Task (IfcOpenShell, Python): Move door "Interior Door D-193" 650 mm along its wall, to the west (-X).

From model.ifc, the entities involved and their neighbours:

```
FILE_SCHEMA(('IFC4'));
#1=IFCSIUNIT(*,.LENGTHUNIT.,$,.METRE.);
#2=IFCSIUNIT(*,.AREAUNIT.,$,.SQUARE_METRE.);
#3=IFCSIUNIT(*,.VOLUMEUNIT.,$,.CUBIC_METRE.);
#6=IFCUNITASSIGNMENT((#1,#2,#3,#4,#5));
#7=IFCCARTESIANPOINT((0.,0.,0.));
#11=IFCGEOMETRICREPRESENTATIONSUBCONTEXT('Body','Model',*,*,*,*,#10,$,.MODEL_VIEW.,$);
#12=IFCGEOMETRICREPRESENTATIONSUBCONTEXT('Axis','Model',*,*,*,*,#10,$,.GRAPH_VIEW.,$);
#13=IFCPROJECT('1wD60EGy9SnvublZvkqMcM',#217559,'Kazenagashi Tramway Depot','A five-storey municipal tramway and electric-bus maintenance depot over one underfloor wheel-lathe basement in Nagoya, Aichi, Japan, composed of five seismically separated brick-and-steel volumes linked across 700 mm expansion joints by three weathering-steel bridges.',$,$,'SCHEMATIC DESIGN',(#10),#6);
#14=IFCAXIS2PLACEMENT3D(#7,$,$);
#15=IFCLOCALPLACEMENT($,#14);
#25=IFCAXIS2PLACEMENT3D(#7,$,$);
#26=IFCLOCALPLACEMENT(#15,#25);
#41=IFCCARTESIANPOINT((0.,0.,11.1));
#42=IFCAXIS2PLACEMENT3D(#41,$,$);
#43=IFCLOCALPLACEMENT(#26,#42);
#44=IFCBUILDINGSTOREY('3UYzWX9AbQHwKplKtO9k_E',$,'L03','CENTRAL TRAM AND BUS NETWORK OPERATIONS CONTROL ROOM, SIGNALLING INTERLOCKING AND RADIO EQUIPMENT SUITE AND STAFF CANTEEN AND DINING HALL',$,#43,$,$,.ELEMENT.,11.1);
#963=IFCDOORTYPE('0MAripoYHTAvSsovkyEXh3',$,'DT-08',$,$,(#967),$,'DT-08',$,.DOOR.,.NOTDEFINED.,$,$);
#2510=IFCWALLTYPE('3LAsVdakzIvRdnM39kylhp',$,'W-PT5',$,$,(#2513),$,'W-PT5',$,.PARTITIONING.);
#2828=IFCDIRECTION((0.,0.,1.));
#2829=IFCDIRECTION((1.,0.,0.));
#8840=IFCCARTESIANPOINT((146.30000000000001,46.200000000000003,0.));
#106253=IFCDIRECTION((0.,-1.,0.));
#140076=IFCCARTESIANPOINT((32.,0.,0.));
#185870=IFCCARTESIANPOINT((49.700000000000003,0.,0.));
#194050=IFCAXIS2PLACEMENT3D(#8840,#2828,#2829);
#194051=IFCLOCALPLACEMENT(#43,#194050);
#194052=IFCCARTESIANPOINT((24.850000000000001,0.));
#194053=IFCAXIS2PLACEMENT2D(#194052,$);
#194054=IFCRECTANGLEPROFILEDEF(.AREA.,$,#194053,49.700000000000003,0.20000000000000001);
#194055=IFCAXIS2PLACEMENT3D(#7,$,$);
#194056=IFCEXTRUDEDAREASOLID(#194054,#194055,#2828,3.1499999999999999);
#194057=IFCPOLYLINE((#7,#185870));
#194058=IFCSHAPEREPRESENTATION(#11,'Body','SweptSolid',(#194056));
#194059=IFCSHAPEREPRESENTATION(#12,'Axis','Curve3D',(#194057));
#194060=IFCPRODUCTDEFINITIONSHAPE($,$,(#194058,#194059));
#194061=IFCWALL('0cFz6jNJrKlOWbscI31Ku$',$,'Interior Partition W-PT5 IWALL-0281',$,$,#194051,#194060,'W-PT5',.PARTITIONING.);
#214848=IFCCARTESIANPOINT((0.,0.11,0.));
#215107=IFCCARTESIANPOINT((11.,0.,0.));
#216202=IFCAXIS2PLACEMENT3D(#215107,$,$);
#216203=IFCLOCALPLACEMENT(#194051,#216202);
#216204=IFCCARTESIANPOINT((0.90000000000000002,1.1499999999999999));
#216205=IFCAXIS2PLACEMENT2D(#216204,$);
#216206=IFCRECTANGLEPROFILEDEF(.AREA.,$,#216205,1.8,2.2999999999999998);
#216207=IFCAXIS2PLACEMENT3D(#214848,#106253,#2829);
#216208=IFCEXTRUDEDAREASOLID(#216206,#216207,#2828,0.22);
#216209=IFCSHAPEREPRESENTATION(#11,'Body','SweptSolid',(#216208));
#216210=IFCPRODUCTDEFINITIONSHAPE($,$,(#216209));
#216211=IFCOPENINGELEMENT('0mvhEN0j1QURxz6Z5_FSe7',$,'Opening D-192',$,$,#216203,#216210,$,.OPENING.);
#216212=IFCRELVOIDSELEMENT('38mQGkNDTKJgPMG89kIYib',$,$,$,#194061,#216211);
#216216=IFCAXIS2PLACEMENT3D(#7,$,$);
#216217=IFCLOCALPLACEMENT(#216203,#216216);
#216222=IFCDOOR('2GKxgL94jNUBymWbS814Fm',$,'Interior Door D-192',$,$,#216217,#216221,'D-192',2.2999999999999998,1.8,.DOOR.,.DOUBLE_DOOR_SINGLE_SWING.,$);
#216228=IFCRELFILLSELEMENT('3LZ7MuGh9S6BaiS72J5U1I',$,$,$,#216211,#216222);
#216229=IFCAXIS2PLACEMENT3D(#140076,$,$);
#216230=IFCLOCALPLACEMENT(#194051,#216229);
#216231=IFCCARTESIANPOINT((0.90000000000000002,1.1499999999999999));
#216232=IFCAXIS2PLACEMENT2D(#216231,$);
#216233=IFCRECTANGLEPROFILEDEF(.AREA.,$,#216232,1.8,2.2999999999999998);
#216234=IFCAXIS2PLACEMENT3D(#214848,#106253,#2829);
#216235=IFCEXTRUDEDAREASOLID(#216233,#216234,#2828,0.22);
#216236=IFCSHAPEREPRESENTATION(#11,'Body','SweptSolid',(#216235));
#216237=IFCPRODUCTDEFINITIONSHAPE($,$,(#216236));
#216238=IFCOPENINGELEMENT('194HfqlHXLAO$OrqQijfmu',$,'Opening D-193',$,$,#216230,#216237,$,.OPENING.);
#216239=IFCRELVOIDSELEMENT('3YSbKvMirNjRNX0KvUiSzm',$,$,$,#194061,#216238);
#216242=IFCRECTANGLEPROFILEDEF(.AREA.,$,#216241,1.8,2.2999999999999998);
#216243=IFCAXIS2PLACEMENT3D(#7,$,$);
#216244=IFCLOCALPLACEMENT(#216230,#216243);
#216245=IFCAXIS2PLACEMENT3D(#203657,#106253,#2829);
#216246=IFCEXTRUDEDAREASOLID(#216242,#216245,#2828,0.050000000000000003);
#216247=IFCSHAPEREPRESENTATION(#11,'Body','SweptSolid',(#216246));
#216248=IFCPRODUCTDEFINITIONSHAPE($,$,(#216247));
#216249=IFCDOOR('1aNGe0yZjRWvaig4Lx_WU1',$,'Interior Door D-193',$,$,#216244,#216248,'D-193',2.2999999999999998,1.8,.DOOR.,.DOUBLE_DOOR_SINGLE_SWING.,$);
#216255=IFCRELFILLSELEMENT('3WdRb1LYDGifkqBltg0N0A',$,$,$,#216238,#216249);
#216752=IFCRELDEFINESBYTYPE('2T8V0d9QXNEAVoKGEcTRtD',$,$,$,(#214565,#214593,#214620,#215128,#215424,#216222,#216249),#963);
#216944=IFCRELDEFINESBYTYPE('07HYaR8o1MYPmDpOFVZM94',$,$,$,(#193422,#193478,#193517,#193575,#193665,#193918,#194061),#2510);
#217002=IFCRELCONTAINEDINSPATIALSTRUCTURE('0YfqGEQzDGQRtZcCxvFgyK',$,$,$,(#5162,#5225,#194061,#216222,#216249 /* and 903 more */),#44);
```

```python
import ifcopenshell
import ifcopenshell.api.geometry
import ifcopenshell.util.placement

model = ifcopenshell.open("model.ifc")

door = model.by_id(216249)
opening = door.FillsVoids[0].RelatingOpeningElement
wall = opening.VoidsElements[0].RelatingBuildingElement

wall_matrix = ifcopenshell.util.placement.get_local_placement(wall.ObjectPlacement)
shift = wall_matrix[:3, 0] * -0.65
before = ifcopenshell.util.placement.get_local_placement(door.ObjectPlacement)[:3, 3].copy()

# The door is placed relative to its opening, so it follows when the opening moves.
matrix = ifcopenshell.util.placement.get_local_placement(opening.ObjectPlacement)
matrix[:3, 3] += shift
ifcopenshell.api.geometry.edit_object_placement(
    model, product=opening, matrix=matrix, is_si=False, should_transform_children=True
)

after = ifcopenshell.util.placement.get_local_placement(door.ObjectPlacement)[:3, 3]
print("door moved by", (after - before).round(3) + 0.0)

model.write("model_rev.ifc")
```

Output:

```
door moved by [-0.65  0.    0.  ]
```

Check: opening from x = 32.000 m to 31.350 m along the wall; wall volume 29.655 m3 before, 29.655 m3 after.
